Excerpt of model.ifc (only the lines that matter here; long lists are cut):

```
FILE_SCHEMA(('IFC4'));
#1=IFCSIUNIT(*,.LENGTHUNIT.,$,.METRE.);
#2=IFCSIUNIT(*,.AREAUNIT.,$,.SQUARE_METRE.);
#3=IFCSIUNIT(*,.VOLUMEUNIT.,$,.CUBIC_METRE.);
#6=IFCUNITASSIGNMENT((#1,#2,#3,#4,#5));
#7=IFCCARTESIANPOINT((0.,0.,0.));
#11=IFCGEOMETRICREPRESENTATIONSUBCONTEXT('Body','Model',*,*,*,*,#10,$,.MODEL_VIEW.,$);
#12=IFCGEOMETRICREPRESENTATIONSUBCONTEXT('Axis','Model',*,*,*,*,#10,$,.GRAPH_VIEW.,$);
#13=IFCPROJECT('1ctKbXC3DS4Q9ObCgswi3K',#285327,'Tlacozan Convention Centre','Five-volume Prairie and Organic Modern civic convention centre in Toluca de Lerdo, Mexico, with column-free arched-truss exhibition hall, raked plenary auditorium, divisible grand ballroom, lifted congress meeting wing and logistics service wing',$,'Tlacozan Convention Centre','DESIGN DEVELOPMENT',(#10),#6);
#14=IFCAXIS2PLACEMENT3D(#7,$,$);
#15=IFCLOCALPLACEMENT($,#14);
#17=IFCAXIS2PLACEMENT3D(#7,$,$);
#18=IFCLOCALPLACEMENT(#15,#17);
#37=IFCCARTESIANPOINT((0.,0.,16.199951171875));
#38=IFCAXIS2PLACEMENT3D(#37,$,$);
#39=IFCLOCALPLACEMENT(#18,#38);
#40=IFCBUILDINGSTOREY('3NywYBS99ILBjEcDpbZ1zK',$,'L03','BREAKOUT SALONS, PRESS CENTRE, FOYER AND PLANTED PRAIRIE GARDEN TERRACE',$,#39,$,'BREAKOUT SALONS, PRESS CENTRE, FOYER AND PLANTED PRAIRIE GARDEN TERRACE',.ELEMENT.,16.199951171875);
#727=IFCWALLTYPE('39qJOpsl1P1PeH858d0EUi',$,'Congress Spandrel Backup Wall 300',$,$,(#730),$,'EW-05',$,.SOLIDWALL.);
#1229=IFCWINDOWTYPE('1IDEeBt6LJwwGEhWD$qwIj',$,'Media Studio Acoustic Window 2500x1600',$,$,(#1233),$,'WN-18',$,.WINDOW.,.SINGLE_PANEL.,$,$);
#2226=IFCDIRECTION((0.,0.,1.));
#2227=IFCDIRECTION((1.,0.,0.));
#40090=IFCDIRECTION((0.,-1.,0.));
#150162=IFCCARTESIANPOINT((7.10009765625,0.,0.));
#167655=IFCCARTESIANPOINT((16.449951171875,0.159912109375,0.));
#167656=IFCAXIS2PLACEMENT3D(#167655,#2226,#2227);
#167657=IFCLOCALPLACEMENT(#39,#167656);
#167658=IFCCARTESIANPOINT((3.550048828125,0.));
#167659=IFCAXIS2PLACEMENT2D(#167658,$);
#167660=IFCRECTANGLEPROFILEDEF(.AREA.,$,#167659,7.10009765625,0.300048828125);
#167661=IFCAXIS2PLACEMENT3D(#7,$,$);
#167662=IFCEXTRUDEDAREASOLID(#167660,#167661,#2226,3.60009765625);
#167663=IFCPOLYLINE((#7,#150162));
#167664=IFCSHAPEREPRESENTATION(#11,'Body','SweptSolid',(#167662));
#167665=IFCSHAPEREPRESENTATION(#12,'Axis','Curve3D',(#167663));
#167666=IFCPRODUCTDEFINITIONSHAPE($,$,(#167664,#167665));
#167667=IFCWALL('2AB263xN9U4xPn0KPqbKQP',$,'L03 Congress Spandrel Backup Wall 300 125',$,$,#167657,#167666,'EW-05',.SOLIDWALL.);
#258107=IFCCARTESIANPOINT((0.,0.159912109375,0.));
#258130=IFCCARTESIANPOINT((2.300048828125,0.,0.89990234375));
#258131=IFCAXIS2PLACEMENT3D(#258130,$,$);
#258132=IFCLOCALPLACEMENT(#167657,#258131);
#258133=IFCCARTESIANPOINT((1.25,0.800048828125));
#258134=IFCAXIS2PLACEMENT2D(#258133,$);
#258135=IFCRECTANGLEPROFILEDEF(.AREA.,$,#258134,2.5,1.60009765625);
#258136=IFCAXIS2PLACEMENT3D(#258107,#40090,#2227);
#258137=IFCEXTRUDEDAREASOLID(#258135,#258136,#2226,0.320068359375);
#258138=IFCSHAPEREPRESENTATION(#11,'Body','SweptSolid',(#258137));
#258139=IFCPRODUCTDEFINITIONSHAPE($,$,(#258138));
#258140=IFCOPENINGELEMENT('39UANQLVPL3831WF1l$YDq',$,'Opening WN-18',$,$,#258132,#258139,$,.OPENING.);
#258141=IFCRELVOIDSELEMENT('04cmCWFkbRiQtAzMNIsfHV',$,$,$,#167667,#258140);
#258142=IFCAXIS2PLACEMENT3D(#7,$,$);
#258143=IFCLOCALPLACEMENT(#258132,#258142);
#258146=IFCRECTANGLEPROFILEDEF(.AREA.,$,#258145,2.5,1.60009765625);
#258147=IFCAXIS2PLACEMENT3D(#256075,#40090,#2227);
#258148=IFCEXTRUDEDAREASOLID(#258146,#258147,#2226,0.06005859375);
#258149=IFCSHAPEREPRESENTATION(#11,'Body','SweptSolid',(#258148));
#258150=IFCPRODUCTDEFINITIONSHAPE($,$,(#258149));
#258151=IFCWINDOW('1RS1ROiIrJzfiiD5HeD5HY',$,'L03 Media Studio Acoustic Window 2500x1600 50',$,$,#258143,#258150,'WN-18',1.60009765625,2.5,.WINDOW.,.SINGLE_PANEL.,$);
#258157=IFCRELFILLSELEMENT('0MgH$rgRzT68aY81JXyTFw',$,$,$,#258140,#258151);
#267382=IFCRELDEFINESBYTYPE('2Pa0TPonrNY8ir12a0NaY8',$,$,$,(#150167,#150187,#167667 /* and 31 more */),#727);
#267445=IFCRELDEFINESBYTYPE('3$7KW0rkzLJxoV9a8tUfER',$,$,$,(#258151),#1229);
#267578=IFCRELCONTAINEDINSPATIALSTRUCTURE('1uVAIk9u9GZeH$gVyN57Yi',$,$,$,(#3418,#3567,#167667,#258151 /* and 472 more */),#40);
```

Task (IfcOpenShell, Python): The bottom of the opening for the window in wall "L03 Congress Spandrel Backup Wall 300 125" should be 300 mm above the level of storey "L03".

```python
import numpy as np
import ifcopenshell
import ifcopenshell.api.geometry
import ifcopenshell.geom
import ifcopenshell.util.element
import ifcopenshell.util.placement
import ifcopenshell.util.shape
import ifcopenshell.util.unit

model = ifcopenshell.open("model.ifc")
unit_scale = ifcopenshell.util.unit.calculate_unit_scale(model)

window = model.by_guid("1RS1ROiIrJzfiiD5HeD5HY")
opening = window.FillsVoids[0].RelatingOpeningElement
storey = ifcopenshell.util.element.get_container(window, ifc_class="IfcBuildingStorey")
level = ifcopenshell.util.placement.get_local_placement(storey.ObjectPlacement)[2, 3]

# The opening's origin need not be at the sill, so measure its lowest point.
shape = ifcopenshell.geom.create_shape(ifcopenshell.geom.settings(), opening)
bottom = ifcopenshell.util.shape.get_shape_bottom_elevation(shape, shape.geometry) / unit_scale
dz = level + 0.3 / unit_scale - bottom

shift = np.array([0.0, 0.0, dz])
# The window is placed relative to its opening, so it follows when the opening moves.
matrix = ifcopenshell.util.placement.get_local_placement(opening.ObjectPlacement)
matrix[:3, 3] += shift
ifcopenshell.api.geometry.edit_object_placement(
    model, product=opening, matrix=matrix, is_si=False, should_transform_children=True
)

print(f"moved by {dz * unit_scale:+.3f} m")

model.write("model_updated.ifc")
```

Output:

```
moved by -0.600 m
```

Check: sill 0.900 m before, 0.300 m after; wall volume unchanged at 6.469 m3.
